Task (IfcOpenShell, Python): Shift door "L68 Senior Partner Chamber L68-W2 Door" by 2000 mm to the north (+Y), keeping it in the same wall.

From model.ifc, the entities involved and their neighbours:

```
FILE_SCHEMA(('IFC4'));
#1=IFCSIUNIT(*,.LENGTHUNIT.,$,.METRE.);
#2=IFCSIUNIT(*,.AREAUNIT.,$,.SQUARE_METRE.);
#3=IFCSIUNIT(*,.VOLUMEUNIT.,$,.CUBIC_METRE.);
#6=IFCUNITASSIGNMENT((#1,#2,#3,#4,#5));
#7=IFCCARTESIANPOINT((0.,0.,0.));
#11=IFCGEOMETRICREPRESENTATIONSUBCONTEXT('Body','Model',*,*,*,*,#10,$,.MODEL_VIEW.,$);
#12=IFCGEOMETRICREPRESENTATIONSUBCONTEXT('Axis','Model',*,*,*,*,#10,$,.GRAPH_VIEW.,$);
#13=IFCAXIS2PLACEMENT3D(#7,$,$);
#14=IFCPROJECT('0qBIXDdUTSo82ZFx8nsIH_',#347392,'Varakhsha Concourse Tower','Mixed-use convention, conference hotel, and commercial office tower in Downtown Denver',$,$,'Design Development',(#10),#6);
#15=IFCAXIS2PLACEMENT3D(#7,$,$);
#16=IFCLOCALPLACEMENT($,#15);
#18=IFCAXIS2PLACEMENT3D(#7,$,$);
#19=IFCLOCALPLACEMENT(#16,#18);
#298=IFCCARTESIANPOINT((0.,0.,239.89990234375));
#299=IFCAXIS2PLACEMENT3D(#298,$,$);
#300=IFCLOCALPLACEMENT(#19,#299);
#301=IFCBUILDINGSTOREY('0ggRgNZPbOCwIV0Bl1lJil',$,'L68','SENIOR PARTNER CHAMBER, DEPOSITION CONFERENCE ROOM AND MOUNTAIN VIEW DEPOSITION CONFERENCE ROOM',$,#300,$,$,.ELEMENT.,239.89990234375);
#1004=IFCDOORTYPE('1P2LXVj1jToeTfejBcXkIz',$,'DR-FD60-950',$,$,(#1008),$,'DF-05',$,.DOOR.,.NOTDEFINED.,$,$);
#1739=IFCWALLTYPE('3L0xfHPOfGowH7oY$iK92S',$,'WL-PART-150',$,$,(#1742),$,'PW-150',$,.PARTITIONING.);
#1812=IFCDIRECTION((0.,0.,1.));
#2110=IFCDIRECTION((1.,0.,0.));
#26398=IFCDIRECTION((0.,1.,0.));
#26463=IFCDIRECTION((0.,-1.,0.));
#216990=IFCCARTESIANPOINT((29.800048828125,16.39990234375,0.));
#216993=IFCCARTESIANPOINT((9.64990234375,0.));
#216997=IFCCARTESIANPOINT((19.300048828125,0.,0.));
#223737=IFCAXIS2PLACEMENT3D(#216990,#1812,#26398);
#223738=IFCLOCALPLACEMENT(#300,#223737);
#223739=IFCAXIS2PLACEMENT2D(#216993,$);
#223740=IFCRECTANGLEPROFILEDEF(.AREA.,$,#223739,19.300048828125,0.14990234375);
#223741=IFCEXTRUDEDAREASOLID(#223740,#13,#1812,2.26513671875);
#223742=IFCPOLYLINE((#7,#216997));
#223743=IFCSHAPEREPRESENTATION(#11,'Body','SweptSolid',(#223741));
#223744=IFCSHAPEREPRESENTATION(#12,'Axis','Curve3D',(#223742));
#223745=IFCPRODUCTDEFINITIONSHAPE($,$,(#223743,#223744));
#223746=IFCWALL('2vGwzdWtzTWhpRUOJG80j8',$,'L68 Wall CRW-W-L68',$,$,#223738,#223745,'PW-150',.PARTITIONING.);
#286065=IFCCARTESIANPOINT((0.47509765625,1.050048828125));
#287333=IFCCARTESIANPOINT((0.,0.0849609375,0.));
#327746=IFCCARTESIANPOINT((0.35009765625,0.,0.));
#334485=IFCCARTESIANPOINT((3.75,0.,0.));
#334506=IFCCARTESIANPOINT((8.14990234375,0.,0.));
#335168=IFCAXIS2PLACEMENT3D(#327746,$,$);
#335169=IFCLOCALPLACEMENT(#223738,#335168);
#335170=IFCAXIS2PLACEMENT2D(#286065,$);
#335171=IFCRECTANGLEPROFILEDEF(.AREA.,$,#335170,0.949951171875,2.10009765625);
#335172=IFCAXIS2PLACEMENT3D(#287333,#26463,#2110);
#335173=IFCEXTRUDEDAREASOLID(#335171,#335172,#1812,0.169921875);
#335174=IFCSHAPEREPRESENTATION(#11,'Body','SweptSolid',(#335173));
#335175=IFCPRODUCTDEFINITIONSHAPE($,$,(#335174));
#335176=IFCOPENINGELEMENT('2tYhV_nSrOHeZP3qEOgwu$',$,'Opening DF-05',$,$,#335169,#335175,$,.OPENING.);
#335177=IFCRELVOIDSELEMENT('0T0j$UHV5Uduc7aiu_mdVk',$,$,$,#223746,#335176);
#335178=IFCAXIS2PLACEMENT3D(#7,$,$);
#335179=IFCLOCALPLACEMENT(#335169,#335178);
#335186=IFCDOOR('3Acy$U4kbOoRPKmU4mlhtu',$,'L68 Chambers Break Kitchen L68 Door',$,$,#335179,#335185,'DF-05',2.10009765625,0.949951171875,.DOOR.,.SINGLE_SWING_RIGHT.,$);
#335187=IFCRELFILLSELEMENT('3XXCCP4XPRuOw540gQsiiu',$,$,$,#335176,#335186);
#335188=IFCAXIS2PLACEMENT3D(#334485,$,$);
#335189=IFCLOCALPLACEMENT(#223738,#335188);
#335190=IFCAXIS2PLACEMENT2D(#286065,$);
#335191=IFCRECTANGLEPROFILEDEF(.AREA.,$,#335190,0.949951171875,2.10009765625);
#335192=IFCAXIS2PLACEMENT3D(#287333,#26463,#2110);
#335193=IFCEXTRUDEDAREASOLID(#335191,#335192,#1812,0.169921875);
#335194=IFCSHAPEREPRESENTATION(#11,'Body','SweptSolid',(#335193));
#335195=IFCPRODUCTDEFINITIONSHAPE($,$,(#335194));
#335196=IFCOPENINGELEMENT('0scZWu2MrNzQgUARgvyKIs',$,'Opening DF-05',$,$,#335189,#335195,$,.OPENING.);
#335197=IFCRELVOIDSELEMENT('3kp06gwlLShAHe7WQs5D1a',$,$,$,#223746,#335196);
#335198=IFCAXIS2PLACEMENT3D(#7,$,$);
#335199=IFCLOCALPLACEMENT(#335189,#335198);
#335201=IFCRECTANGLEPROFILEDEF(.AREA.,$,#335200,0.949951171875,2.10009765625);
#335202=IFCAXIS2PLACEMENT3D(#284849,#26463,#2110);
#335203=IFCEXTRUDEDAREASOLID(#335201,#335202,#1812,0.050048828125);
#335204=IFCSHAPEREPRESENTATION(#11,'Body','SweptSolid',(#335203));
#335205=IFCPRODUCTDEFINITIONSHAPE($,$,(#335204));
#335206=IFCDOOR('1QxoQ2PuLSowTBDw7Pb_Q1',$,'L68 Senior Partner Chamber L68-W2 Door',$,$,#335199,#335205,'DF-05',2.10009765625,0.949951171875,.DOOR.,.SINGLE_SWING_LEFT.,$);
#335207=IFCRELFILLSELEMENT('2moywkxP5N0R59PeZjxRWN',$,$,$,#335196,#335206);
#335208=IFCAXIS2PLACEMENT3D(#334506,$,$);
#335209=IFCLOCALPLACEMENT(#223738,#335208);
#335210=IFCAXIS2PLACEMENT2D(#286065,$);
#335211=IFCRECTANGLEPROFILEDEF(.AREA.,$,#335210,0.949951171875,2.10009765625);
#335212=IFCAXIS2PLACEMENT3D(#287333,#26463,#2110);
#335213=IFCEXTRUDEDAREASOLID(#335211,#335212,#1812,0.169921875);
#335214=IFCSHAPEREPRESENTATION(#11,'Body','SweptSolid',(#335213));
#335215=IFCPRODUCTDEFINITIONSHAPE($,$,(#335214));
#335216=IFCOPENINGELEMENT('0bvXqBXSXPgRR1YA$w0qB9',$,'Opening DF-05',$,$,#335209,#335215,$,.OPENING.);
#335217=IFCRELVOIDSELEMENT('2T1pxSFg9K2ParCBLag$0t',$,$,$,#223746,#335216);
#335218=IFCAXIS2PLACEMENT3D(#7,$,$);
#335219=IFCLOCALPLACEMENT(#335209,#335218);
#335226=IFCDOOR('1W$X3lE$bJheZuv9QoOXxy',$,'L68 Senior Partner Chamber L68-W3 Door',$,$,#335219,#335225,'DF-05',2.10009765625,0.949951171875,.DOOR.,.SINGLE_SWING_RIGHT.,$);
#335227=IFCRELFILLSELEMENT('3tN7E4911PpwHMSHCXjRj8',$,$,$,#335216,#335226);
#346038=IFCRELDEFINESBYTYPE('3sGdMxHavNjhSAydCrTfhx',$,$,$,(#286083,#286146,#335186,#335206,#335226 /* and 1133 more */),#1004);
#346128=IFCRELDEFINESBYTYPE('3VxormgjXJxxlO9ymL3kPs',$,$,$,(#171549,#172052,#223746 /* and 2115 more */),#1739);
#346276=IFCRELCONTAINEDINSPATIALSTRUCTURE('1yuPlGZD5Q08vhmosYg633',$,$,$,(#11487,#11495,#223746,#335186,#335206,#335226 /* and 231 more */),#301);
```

```python
import ifcopenshell
import ifcopenshell.api.geometry
import ifcopenshell.util.placement

model = ifcopenshell.open("model.ifc")

door = model.by_id(335206)
opening = door.FillsVoids[0].RelatingOpeningElement
wall = opening.VoidsElements[0].RelatingBuildingElement

wall_matrix = ifcopenshell.util.placement.get_local_placement(wall.ObjectPlacement)
shift = wall_matrix[:3, 0] * 2.0
before = ifcopenshell.util.placement.get_local_placement(door.ObjectPlacement)[:3, 3].copy()

# The door is placed relative to its opening, so it follows when the opening moves.
matrix = ifcopenshell.util.placement.get_local_placement(opening.ObjectPlacement)
matrix[:3, 3] += shift
ifcopenshell.api.geometry.edit_object_placement(
    model, product=opening, matrix=matrix, is_si=False, should_transform_children=True
)

after = ifcopenshell.util.placement.get_local_placement(door.ObjectPlacement)[:3, 3]
print("door moved by", (after - before).round(3) + 0.0)

model.write("model_edited.ifc")
```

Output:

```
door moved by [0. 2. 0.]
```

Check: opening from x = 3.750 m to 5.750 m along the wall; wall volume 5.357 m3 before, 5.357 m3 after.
